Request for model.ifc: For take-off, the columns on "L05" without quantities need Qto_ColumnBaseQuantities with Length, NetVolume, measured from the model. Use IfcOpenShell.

First a look at what the model holds.

```python
import ifcopenshell
import ifcopenshell.util.element
import ifcopenshell.util.unit

model = ifcopenshell.open("model.ifc")
print(model.schema)
for unit_type in ("LENGTHUNIT", "AREAUNIT", "VOLUMEUNIT"):
    print(unit_type, ifcopenshell.util.unit.calculate_unit_scale(model, unit_type))
storey = next(s for s in model.by_type("IfcBuildingStorey") if s.Name == "L05")
columns = [e for e in ifcopenshell.util.element.get_decomposition(storey) if e.is_a("IfcColumn")]
for e in sorted(columns, key=lambda e: e.id()):
    print(e.id(), e.is_a(), e.Name, list(ifcopenshell.util.element.get_psets(e, qtos_only=True)), sep=" | ")
```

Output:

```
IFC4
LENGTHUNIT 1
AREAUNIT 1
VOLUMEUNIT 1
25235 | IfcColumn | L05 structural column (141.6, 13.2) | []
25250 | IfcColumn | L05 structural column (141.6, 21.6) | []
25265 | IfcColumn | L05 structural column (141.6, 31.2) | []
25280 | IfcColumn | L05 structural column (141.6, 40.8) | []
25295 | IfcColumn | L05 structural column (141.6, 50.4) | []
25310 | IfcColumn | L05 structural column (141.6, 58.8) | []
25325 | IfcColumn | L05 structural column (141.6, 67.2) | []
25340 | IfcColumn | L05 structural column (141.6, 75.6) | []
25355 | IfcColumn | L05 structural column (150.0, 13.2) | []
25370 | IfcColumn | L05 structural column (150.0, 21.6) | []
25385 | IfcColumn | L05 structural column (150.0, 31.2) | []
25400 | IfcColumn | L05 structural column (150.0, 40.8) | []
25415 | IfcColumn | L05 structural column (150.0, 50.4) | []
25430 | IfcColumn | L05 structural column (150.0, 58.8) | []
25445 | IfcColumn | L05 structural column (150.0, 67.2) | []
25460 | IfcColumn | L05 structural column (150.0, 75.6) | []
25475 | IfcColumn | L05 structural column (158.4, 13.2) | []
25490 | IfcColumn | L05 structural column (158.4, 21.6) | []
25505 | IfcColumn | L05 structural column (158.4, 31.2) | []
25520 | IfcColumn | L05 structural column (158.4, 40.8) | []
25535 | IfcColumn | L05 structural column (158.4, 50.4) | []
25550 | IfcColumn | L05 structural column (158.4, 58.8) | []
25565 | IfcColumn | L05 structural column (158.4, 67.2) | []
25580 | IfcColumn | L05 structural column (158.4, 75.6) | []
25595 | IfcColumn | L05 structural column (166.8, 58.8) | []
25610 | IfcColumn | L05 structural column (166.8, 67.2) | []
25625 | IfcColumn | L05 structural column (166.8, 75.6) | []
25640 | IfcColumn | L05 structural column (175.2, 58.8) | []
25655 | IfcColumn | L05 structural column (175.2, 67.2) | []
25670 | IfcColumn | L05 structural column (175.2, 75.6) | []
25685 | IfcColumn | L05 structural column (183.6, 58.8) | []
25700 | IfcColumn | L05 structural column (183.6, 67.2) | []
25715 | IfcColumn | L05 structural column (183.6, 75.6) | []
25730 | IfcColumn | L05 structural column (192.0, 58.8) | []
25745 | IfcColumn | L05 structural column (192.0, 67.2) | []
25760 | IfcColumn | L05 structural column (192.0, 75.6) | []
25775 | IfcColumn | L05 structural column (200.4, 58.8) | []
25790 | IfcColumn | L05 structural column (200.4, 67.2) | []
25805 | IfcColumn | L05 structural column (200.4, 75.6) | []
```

```python
import ifcopenshell
import ifcopenshell.api.pset
import ifcopenshell.geom
import ifcopenshell.util.element
import ifcopenshell.util.shape
import ifcopenshell.util.unit

model = ifcopenshell.open("model.ifc")
unit_scale = ifcopenshell.util.unit.calculate_unit_scale(model)
volume_scale = ifcopenshell.util.unit.calculate_unit_scale(model, "VOLUMEUNIT")
settings = ifcopenshell.geom.settings()

storey = next(s for s in model.by_type("IfcBuildingStorey") if s.Name == "L05")
columns = [e for e in ifcopenshell.util.element.get_decomposition(storey) if e.is_a("IfcColumn")]

for e in sorted(columns, key=lambda e: e.id()):
    if ifcopenshell.util.element.get_psets(e, qtos_only=True, should_inherit=False):
        continue
    # Geometry comes back in metres, in the element's own axes.
    shape = ifcopenshell.geom.create_shape(settings, e)
    values = {
        "Length": ifcopenshell.util.shape.get_z(shape.geometry) / unit_scale,
        "NetVolume": ifcopenshell.util.shape.get_volume(shape.geometry) / volume_scale,
    }
    qto = ifcopenshell.api.pset.add_qto(model, product=e, name="Qto_ColumnBaseQuantities")
    ifcopenshell.api.pset.edit_qto(model, qto=qto, properties=values)
    print(e.id(), {k: round(v, 3) for k, v in values.items()})

model.write("model-out.ifc")
```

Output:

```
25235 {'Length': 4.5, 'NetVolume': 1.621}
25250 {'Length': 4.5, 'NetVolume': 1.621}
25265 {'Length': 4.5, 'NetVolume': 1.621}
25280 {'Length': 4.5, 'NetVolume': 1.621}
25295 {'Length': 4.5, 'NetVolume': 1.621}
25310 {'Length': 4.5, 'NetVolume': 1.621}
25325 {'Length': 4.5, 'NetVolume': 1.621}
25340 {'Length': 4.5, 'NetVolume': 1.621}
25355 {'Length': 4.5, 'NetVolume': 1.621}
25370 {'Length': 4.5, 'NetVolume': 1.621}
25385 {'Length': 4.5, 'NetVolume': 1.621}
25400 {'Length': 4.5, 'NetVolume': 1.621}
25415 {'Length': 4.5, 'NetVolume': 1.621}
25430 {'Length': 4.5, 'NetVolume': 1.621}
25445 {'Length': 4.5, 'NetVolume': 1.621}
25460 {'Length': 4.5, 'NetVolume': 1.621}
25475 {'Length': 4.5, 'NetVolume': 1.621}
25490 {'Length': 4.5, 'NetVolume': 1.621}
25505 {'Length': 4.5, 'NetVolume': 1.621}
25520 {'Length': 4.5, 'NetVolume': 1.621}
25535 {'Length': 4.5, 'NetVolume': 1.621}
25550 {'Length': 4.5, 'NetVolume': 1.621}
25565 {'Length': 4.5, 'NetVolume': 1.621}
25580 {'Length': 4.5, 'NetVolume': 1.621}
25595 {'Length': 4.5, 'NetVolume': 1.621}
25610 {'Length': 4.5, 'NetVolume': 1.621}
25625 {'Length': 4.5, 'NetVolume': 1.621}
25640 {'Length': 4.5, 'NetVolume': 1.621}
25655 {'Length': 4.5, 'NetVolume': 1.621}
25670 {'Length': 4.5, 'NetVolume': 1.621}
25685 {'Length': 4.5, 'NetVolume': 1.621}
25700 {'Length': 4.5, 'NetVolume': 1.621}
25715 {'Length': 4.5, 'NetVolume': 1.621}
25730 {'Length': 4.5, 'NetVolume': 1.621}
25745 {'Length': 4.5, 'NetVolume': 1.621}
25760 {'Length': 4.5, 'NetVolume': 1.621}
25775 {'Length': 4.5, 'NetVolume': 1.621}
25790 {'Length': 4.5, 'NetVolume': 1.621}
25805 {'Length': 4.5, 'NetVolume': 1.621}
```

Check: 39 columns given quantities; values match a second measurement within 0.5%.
